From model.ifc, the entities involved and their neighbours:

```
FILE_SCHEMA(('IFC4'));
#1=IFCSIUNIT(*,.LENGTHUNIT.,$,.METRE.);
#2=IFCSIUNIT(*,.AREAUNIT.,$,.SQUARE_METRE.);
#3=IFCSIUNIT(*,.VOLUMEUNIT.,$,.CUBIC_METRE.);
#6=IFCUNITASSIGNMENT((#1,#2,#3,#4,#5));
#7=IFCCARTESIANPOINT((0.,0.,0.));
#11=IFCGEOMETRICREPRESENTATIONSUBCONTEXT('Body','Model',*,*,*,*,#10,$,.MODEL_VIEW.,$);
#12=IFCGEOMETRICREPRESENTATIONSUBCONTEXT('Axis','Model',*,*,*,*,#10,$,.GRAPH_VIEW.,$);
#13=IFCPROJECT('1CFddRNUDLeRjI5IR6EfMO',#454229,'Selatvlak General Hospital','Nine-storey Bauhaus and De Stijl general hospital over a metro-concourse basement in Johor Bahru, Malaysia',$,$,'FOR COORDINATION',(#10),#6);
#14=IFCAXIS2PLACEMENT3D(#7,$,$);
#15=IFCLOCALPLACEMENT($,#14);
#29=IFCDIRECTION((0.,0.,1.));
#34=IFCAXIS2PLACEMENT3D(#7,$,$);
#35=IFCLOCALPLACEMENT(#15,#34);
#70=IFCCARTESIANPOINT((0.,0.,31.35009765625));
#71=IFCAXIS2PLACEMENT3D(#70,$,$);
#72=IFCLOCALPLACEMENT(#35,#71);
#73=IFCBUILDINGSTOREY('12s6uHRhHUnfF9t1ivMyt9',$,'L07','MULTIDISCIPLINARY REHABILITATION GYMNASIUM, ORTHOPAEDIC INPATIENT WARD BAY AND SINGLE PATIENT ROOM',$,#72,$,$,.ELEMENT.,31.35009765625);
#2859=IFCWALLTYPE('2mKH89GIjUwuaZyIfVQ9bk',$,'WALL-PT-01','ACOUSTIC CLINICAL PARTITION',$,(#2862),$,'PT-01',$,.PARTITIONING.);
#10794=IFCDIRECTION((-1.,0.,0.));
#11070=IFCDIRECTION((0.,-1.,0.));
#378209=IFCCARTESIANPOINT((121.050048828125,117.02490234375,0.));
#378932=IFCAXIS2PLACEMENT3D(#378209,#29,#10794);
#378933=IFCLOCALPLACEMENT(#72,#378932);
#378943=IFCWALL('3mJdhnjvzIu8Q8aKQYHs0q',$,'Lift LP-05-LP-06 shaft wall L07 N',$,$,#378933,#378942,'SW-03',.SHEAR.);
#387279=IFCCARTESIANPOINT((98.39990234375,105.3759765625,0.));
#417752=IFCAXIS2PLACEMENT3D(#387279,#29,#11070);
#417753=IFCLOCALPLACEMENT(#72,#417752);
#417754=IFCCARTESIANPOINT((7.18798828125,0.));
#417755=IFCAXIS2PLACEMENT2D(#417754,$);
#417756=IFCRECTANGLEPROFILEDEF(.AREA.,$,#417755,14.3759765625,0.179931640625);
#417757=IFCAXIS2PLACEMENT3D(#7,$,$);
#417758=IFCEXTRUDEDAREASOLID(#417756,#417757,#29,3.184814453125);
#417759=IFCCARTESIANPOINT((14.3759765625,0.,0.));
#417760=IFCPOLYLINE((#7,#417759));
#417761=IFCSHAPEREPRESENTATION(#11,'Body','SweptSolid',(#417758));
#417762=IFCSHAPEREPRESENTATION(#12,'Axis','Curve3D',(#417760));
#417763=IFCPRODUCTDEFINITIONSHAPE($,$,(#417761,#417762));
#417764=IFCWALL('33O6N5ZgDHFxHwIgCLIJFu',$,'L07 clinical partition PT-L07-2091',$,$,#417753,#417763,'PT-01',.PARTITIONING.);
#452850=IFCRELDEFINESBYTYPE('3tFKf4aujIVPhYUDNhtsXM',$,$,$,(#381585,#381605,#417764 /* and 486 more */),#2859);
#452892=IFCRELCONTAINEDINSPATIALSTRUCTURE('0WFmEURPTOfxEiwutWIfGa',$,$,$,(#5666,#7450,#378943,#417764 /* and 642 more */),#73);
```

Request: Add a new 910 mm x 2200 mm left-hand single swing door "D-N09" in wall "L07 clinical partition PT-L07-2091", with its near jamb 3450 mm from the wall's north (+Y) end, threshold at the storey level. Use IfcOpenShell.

```python
import numpy as np
import ifcopenshell
import ifcopenshell.api.feature
import ifcopenshell.api.geometry
import ifcopenshell.api.root
import ifcopenshell.api.spatial
import ifcopenshell.geom
import ifcopenshell.util.element
import ifcopenshell.util.placement
import ifcopenshell.util.representation
import ifcopenshell.util.shape
import ifcopenshell.util.unit

model = ifcopenshell.open("model.ifc")
unit_scale = ifcopenshell.util.unit.calculate_unit_scale(model)
settings = ifcopenshell.geom.settings()


def volume(element):
    """Net volume in cubic metres, openings subtracted."""
    shape = ifcopenshell.geom.create_shape(settings, element)
    return ifcopenshell.util.shape.get_volume(shape.geometry)


wall = model.by_guid("33O6N5ZgDHFxHwIgCLIJFu")
storey = ifcopenshell.util.element.get_container(wall, ifc_class="IfcBuildingStorey")
context = ifcopenshell.util.representation.get_context(model, "Model", "Body", "MODEL_VIEW")
before = volume(wall)

width, height, from_end, sill = 0.91, 2.2, 3.45, 0.0  # metres

# The wall runs along its own X axis, and the end named is its -X end.
wall_shape = ifcopenshell.geom.create_shape(settings, wall)
x, y, z = ifcopenshell.util.shape.get_vertices(wall_shape.geometry).T
start = x.min() + from_end
face, thickness = float(y.min()), float(y.max() - y.min())
wall_matrix = ifcopenshell.util.placement.get_local_placement(wall.ObjectPlacement)
level = ifcopenshell.util.placement.get_local_placement(storey.ObjectPlacement)[2, 3]


def in_wall(x, y):
    """Placement at x, y metres in the wall's axes, at sill height."""
    matrix = wall_matrix.copy()
    matrix[:, 3] = wall_matrix @ np.array([x / unit_scale, y / unit_scale, 0.0, 1.0])
    matrix[2, 3] = level + sill / unit_scale
    return matrix


# Opening: a box that overshoots both wall faces by 50 mm.
opening = ifcopenshell.api.root.create_entity(model, ifc_class="IfcOpeningElement", predefined_type="OPENING")
box = ifcopenshell.api.geometry.add_wall_representation(
    model, context=context, length=width, height=height, thickness=thickness + 0.1
)
ifcopenshell.api.geometry.assign_representation(model, product=opening, representation=box)
ifcopenshell.api.geometry.edit_object_placement(model, product=opening, matrix=in_wall(start, face - 0.05), is_si=False)
ifcopenshell.api.feature.add_feature(model, feature=opening, element=wall)

door = ifcopenshell.api.root.create_entity(model, ifc_class="IfcDoor", name="D-N09", predefined_type="DOOR")
door.OverallWidth, door.OverallHeight = width / unit_scale, height / unit_scale
door.OperationType = "SINGLE_SWING_LEFT"
body = ifcopenshell.api.geometry.add_door_representation(
    model,
    context=context,
    overall_width=door.OverallWidth,
    overall_height=door.OverallHeight,
    operation_type="SINGLE_SWING_LEFT",
    lining_properties={"LiningDepth": thickness / unit_scale, "ThresholdDepth": thickness / unit_scale},
)
ifcopenshell.api.geometry.assign_representation(model, product=door, representation=body)
ifcopenshell.api.spatial.assign_container(model, products=[door], relating_structure=storey)
ifcopenshell.api.feature.add_filling(model, opening=opening, element=door)

# The lining spans the wall, so the door starts at the wall face.
ifcopenshell.api.geometry.edit_object_placement(model, product=door, matrix=in_wall(start, face), is_si=False)

after = volume(wall)

print(f"wall volume {before:.3f} -> {after:.3f} m3")

model.write("model-out.ifc")
```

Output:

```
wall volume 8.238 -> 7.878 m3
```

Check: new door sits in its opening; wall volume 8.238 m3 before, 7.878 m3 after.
